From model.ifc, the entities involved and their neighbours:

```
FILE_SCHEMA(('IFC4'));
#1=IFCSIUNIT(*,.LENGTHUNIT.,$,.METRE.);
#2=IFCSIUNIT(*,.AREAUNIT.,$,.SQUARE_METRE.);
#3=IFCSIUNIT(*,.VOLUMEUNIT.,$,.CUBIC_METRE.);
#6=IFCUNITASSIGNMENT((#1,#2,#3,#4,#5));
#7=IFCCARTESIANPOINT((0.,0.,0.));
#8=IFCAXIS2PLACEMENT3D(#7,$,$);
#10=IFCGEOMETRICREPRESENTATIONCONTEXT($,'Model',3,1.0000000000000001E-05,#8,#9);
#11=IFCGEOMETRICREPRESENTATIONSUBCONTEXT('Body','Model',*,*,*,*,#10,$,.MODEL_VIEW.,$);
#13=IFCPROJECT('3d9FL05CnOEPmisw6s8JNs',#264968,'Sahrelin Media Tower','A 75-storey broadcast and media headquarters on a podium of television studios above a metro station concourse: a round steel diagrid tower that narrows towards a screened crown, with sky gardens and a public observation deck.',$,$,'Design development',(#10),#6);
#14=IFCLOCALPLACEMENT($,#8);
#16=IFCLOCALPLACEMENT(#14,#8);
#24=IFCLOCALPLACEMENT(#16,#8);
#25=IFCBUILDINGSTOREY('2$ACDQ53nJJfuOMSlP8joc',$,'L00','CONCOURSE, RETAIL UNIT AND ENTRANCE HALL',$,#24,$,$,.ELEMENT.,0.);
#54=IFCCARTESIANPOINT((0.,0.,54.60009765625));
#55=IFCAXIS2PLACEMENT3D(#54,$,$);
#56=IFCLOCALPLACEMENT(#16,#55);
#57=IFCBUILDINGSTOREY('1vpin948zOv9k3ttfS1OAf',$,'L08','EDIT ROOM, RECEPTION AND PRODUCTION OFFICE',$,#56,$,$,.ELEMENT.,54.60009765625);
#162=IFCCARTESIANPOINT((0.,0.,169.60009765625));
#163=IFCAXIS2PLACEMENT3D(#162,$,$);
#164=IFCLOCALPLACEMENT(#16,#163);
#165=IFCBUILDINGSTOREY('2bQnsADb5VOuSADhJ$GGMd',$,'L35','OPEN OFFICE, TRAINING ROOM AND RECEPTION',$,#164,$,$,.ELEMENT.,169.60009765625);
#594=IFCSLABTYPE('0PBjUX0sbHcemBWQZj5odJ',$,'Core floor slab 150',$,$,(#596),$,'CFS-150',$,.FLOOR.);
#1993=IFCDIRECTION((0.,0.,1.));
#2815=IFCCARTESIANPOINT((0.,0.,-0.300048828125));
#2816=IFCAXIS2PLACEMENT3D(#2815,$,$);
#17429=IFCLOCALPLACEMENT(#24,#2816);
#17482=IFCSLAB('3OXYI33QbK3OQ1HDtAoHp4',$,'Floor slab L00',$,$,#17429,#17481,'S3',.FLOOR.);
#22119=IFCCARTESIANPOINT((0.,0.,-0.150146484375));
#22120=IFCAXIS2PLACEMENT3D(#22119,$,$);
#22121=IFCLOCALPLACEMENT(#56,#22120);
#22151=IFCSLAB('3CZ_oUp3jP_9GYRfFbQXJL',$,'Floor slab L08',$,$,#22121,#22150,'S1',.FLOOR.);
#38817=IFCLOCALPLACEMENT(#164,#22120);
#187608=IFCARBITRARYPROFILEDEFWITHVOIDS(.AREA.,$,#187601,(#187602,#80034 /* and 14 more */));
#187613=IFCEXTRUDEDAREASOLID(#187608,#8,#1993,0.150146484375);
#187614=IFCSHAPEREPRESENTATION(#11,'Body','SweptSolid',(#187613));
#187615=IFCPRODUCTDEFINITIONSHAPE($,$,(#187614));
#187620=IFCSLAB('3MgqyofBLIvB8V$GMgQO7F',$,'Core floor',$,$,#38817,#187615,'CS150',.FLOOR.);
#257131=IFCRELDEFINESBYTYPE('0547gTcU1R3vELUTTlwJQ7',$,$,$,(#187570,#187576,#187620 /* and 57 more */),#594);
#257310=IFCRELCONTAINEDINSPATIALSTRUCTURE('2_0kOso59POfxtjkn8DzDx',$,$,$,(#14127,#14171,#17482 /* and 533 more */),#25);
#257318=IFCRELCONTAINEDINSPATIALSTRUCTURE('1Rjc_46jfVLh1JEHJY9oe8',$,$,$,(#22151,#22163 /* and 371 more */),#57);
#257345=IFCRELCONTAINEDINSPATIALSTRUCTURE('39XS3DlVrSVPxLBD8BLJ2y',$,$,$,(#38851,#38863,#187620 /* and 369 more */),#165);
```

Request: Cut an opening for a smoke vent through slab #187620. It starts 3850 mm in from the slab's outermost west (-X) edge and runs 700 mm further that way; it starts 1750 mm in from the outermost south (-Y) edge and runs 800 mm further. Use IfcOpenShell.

```python
import numpy as np
import ifcopenshell
import ifcopenshell.api.feature
import ifcopenshell.api.geometry
import ifcopenshell.api.root
import ifcopenshell.geom
import ifcopenshell.util.placement
import ifcopenshell.util.representation
import ifcopenshell.util.shape
import ifcopenshell.util.unit

model = ifcopenshell.open("model.ifc")
unit_scale = ifcopenshell.util.unit.calculate_unit_scale(model)
settings = ifcopenshell.geom.settings()


def volume(element):
    """Net volume in cubic metres, openings subtracted."""
    shape = ifcopenshell.geom.create_shape(settings, element)
    return ifcopenshell.util.shape.get_volume(shape.geometry)


slab = model.by_guid("3MgqyofBLIvB8V$GMgQO7F")
before = volume(slab)

# Extent in the slab's own axes, in metres. The edges named are its -X and -Y sides.
slab_shape = ifcopenshell.geom.create_shape(settings, slab)
vertices = ifcopenshell.util.shape.get_vertices(slab_shape.geometry)
x_min, y_min, bottom = vertices.min(axis=0)
top = vertices[:, 2].max()

opening = ifcopenshell.api.root.create_entity(model, ifc_class="IfcOpeningElement", name="Smoke vent opening", predefined_type="OPENING")
context = ifcopenshell.util.representation.get_context(model, "Model", "Body", "MODEL_VIEW")
width, depth = 0.7, 0.8
outline = [(0.0, 0.0), (width, 0.0), (width, depth), (0.0, depth), (0.0, 0.0)]
# Overshoot both faces by 50 mm so the cut is clean.
shape = ifcopenshell.api.geometry.add_slab_representation(
    model, context=context, depth=top - bottom + 0.1, polyline=outline
)
ifcopenshell.api.geometry.assign_representation(model, product=opening, representation=shape)

matrix = ifcopenshell.util.placement.get_local_placement(slab.ObjectPlacement)
matrix[:, 3] = matrix @ np.append(np.array([x_min + 3.85, y_min + 1.75, bottom - 0.05]) / unit_scale, 1.0)
ifcopenshell.api.geometry.edit_object_placement(model, product=opening, matrix=matrix, is_si=False)
ifcopenshell.api.feature.add_feature(model, feature=opening, element=slab)

after = volume(slab)

print(f"slab volume {before:.3f} -> {after:.3f} m3")

model.write("model_edited.ifc")
```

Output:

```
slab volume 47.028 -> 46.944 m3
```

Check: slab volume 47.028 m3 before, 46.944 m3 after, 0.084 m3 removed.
